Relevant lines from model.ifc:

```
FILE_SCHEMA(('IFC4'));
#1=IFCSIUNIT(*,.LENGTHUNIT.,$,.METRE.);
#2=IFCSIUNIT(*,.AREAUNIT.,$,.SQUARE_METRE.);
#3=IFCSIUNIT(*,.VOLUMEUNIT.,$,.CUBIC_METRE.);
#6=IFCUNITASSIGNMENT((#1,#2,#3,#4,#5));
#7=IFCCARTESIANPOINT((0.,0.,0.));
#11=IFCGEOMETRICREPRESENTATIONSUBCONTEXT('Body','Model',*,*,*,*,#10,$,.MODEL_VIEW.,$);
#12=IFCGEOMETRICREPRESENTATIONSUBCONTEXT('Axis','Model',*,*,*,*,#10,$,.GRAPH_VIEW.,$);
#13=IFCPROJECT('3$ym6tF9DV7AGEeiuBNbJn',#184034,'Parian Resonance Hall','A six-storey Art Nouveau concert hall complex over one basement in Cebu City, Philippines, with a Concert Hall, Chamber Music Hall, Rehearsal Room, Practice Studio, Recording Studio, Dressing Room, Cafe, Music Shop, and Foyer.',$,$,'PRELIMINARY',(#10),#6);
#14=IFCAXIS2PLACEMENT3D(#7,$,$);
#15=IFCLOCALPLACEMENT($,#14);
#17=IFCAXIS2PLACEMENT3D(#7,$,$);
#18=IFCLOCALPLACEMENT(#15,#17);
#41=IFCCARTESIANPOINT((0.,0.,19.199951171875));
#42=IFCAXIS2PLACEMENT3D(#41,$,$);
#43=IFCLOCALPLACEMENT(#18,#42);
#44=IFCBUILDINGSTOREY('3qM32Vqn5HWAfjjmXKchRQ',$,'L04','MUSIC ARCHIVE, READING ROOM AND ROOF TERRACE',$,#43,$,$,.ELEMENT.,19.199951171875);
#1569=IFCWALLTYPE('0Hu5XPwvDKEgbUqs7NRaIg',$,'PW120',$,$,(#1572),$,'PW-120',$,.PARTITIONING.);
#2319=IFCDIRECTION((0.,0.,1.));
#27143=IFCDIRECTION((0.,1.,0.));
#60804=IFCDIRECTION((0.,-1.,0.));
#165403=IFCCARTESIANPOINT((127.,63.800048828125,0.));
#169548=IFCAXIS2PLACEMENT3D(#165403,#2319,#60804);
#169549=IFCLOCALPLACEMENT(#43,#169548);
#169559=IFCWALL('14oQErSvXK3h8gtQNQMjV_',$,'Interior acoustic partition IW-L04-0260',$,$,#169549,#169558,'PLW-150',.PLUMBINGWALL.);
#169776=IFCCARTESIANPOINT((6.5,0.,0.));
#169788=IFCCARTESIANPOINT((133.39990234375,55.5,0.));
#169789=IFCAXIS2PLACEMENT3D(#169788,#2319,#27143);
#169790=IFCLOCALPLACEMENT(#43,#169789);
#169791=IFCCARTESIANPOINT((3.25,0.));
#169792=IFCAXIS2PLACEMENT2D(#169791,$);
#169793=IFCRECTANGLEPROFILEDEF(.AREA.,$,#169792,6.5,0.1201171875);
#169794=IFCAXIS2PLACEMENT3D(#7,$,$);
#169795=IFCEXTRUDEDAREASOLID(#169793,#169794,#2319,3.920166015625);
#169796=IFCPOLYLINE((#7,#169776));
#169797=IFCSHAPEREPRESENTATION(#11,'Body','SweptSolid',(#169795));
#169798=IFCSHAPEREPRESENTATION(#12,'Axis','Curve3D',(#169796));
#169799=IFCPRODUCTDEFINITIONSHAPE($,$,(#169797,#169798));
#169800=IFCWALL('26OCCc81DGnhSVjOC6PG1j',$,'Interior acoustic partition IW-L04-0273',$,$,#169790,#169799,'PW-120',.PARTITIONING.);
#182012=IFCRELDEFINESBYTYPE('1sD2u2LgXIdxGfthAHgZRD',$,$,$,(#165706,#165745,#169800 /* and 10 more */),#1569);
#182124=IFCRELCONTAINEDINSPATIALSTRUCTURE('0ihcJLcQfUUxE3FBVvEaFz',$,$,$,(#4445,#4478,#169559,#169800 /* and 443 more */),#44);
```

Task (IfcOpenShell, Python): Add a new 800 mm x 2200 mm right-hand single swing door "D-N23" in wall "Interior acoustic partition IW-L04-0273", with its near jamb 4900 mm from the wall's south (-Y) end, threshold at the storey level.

```python
import numpy as np
import ifcopenshell
import ifcopenshell.api.feature
import ifcopenshell.api.geometry
import ifcopenshell.api.root
import ifcopenshell.api.spatial
import ifcopenshell.geom
import ifcopenshell.util.element
import ifcopenshell.util.placement
import ifcopenshell.util.representation
import ifcopenshell.util.shape
import ifcopenshell.util.unit

model = ifcopenshell.open("model.ifc")
unit_scale = ifcopenshell.util.unit.calculate_unit_scale(model)
settings = ifcopenshell.geom.settings()


def volume(element):
    """Net volume in cubic metres, openings subtracted."""
    shape = ifcopenshell.geom.create_shape(settings, element)
    return ifcopenshell.util.shape.get_volume(shape.geometry)


wall = model.by_guid("26OCCc81DGnhSVjOC6PG1j")
storey = ifcopenshell.util.element.get_container(wall, ifc_class="IfcBuildingStorey")
context = ifcopenshell.util.representation.get_context(model, "Model", "Body", "MODEL_VIEW")
before = volume(wall)

width, height, from_end, sill = 0.8, 2.2, 4.9, 0.0  # metres

# The wall runs along its own X axis, and the end named is its -X end.
wall_shape = ifcopenshell.geom.create_shape(settings, wall)
x, y, z = ifcopenshell.util.shape.get_vertices(wall_shape.geometry).T
start = x.min() + from_end
face, thickness = float(y.min()), float(y.max() - y.min())
wall_matrix = ifcopenshell.util.placement.get_local_placement(wall.ObjectPlacement)
level = ifcopenshell.util.placement.get_local_placement(storey.ObjectPlacement)[2, 3]


def in_wall(x, y):
    """Placement at x, y metres in the wall's axes, at sill height."""
    matrix = wall_matrix.copy()
    matrix[:, 3] = wall_matrix @ np.array([x / unit_scale, y / unit_scale, 0.0, 1.0])
    matrix[2, 3] = level + sill / unit_scale
    return matrix


# Opening: a box that overshoots both wall faces by 50 mm.
opening = ifcopenshell.api.root.create_entity(model, ifc_class="IfcOpeningElement", predefined_type="OPENING")
box = ifcopenshell.api.geometry.add_wall_representation(
    model, context=context, length=width, height=height, thickness=thickness + 0.1
)
ifcopenshell.api.geometry.assign_representation(model, product=opening, representation=box)
ifcopenshell.api.geometry.edit_object_placement(model, product=opening, matrix=in_wall(start, face - 0.05), is_si=False)
ifcopenshell.api.feature.add_feature(model, feature=opening, element=wall)

door = ifcopenshell.api.root.create_entity(model, ifc_class="IfcDoor", name="D-N23", predefined_type="DOOR")
door.OverallWidth, door.OverallHeight = width / unit_scale, height / unit_scale
door.OperationType = "SINGLE_SWING_RIGHT"
body = ifcopenshell.api.geometry.add_door_representation(
    model,
    context=context,
    overall_width=door.OverallWidth,
    overall_height=door.OverallHeight,
    operation_type="SINGLE_SWING_RIGHT",
    lining_properties={"LiningDepth": thickness / unit_scale, "ThresholdDepth": thickness / unit_scale},
)
ifcopenshell.api.geometry.assign_representation(model, product=door, representation=body)
ifcopenshell.api.spatial.assign_container(model, products=[door], relating_structure=storey)
ifcopenshell.api.feature.add_filling(model, opening=opening, element=door)

# The lining spans the wall, so the door starts at the wall face.
ifcopenshell.api.geometry.edit_object_placement(model, product=door, matrix=in_wall(start, face), is_si=False)

after = volume(wall)

print(f"wall volume {before:.3f} -> {after:.3f} m3")

model.write("model_v2.ifc")
```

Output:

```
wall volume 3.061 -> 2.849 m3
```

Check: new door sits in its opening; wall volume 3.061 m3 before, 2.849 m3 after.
